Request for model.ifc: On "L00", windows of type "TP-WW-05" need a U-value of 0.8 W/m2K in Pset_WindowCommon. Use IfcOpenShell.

First a look at what the model holds.

```python
import ifcopenshell
import ifcopenshell.util.element

model = ifcopenshell.open("model.ifc")
print(model.schema)
storey = next(s for s in model.by_type("IfcBuildingStorey") if s.Name == "L00")
windows = [e for e in ifcopenshell.util.element.get_decomposition(storey) if e.is_a("IfcWindow")]
seen = {}
for e in windows:
    element_type = ifcopenshell.util.element.get_type(e)
    key = (element_type.Name if element_type != e and element_type else None, ifcopenshell.util.element.get_pset(e, "Pset_WindowCommon", "ThermalTransmittance"))
    seen[key] = seen.get(key, 0) + 1
for (name, value), count in sorted(seen.items(), key=str):
    print(count, "x", name, "|", value)
```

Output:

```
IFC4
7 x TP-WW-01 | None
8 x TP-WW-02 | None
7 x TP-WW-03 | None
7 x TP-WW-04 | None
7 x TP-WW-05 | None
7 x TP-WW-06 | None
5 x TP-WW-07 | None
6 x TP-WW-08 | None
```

```python
import ifcopenshell
import ifcopenshell.api.pset
import ifcopenshell.util.element

model = ifcopenshell.open("model.ifc")

storey = next(s for s in model.by_type("IfcBuildingStorey") if s.Name == "L00")
windows = [e for e in ifcopenshell.util.element.get_decomposition(storey) if e.is_a("IfcWindow")]

count = 0
for e in windows:
    element_type = ifcopenshell.util.element.get_type(e)
    if element_type in (None, e) or element_type.Name != "TP-WW-05":
        continue
    # add_pset returns the element's existing set when there is one.
    pset = ifcopenshell.api.pset.add_pset(model, product=e, name="Pset_WindowCommon")
    ifcopenshell.api.pset.edit_pset(model, pset=pset, properties={"ThermalTransmittance": 0.8})
    count += 1

print(count, "windows updated")

model.write("model_updated.ifc")
```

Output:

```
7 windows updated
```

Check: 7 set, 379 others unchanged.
